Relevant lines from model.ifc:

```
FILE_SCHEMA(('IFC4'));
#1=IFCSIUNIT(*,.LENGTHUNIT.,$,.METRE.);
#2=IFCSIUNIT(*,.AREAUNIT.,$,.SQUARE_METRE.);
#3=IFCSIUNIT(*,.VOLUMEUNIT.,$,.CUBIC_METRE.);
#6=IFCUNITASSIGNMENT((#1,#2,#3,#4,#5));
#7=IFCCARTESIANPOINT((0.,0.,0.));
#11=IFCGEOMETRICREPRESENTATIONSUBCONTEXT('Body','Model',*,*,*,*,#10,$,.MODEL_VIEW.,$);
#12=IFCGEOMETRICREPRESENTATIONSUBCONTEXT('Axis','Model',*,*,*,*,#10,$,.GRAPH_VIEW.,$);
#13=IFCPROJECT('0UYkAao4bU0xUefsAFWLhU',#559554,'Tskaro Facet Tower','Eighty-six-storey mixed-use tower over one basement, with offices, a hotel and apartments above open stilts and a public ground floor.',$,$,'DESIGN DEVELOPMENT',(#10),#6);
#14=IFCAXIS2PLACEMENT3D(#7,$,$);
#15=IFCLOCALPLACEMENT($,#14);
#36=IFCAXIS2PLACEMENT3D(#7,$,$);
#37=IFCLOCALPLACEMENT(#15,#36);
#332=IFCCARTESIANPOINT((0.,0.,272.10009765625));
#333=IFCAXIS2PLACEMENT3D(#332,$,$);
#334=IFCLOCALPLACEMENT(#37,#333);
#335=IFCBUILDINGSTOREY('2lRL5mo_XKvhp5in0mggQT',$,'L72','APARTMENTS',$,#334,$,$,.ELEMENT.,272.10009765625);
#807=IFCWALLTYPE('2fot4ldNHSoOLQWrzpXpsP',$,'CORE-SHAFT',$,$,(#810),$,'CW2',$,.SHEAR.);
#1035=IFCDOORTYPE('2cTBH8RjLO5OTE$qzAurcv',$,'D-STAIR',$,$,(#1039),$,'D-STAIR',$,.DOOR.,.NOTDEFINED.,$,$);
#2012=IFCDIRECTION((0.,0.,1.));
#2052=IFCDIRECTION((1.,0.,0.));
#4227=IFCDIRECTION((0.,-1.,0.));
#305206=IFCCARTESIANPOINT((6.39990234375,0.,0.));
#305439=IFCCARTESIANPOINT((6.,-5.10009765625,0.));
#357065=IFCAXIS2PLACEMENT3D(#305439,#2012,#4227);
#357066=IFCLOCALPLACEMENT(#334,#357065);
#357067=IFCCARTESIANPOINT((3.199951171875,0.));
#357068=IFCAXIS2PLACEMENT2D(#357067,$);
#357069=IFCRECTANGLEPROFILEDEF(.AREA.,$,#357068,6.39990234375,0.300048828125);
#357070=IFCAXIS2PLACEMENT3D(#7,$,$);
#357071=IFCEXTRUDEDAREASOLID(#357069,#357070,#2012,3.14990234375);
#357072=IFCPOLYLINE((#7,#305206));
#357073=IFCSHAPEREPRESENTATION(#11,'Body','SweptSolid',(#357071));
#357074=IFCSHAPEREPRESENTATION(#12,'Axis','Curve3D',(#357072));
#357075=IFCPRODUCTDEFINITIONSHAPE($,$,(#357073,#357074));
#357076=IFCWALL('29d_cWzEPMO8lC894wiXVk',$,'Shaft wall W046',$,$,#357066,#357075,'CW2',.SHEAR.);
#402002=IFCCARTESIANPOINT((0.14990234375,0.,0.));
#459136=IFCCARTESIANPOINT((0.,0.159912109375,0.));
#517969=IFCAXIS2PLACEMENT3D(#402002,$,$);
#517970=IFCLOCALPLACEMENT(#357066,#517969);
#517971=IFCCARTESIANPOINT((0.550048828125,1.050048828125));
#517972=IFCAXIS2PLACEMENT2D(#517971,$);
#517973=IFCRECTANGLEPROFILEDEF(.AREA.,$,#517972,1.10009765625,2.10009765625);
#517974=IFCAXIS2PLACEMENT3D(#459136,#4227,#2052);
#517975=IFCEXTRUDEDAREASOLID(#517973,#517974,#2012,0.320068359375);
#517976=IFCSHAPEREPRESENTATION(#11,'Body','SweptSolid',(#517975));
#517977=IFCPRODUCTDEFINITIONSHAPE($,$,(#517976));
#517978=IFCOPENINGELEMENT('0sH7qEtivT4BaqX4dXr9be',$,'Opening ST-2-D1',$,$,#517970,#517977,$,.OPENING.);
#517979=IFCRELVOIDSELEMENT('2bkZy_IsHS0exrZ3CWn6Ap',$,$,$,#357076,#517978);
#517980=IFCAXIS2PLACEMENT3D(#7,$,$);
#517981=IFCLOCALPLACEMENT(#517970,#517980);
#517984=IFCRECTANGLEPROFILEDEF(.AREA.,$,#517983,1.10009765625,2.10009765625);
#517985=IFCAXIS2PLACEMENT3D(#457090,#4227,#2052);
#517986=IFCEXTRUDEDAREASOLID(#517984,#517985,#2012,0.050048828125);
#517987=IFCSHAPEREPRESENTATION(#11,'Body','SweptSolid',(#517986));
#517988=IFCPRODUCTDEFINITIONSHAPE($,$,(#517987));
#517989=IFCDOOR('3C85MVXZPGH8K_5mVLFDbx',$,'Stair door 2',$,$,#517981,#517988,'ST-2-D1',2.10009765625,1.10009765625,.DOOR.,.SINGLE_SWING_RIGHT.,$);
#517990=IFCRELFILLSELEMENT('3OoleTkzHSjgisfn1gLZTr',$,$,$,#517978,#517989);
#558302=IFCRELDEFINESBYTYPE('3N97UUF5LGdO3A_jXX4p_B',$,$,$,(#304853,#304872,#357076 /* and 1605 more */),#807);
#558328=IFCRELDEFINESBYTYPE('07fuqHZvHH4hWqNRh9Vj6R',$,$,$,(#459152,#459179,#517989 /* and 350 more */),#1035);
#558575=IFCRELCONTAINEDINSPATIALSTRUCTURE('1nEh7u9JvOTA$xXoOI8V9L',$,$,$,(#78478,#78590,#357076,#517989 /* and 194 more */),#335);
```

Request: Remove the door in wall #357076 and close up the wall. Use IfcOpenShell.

```python
import ifcopenshell
import ifcopenshell.api.feature
import ifcopenshell.api.root
import ifcopenshell.geom
import ifcopenshell.util.shape

model = ifcopenshell.open("model.ifc")
settings = ifcopenshell.geom.settings()


def volume(element):
    """Net volume in cubic metres, openings subtracted."""
    shape = ifcopenshell.geom.create_shape(settings, element)
    return ifcopenshell.util.shape.get_volume(shape.geometry)


door = model.by_id(517989)
opening = door.FillsVoids[0].RelatingOpeningElement
wall = opening.VoidsElements[0].RelatingBuildingElement
before = volume(wall)

ifcopenshell.api.root.remove_product(model, product=door)
ifcopenshell.api.feature.remove_feature(model, feature=opening)

after = volume(wall)

print(f"wall volume {before:.3f} -> {after:.3f} m3")

model.write("model_updated.ifc")
```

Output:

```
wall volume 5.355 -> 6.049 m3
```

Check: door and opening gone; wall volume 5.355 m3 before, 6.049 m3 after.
